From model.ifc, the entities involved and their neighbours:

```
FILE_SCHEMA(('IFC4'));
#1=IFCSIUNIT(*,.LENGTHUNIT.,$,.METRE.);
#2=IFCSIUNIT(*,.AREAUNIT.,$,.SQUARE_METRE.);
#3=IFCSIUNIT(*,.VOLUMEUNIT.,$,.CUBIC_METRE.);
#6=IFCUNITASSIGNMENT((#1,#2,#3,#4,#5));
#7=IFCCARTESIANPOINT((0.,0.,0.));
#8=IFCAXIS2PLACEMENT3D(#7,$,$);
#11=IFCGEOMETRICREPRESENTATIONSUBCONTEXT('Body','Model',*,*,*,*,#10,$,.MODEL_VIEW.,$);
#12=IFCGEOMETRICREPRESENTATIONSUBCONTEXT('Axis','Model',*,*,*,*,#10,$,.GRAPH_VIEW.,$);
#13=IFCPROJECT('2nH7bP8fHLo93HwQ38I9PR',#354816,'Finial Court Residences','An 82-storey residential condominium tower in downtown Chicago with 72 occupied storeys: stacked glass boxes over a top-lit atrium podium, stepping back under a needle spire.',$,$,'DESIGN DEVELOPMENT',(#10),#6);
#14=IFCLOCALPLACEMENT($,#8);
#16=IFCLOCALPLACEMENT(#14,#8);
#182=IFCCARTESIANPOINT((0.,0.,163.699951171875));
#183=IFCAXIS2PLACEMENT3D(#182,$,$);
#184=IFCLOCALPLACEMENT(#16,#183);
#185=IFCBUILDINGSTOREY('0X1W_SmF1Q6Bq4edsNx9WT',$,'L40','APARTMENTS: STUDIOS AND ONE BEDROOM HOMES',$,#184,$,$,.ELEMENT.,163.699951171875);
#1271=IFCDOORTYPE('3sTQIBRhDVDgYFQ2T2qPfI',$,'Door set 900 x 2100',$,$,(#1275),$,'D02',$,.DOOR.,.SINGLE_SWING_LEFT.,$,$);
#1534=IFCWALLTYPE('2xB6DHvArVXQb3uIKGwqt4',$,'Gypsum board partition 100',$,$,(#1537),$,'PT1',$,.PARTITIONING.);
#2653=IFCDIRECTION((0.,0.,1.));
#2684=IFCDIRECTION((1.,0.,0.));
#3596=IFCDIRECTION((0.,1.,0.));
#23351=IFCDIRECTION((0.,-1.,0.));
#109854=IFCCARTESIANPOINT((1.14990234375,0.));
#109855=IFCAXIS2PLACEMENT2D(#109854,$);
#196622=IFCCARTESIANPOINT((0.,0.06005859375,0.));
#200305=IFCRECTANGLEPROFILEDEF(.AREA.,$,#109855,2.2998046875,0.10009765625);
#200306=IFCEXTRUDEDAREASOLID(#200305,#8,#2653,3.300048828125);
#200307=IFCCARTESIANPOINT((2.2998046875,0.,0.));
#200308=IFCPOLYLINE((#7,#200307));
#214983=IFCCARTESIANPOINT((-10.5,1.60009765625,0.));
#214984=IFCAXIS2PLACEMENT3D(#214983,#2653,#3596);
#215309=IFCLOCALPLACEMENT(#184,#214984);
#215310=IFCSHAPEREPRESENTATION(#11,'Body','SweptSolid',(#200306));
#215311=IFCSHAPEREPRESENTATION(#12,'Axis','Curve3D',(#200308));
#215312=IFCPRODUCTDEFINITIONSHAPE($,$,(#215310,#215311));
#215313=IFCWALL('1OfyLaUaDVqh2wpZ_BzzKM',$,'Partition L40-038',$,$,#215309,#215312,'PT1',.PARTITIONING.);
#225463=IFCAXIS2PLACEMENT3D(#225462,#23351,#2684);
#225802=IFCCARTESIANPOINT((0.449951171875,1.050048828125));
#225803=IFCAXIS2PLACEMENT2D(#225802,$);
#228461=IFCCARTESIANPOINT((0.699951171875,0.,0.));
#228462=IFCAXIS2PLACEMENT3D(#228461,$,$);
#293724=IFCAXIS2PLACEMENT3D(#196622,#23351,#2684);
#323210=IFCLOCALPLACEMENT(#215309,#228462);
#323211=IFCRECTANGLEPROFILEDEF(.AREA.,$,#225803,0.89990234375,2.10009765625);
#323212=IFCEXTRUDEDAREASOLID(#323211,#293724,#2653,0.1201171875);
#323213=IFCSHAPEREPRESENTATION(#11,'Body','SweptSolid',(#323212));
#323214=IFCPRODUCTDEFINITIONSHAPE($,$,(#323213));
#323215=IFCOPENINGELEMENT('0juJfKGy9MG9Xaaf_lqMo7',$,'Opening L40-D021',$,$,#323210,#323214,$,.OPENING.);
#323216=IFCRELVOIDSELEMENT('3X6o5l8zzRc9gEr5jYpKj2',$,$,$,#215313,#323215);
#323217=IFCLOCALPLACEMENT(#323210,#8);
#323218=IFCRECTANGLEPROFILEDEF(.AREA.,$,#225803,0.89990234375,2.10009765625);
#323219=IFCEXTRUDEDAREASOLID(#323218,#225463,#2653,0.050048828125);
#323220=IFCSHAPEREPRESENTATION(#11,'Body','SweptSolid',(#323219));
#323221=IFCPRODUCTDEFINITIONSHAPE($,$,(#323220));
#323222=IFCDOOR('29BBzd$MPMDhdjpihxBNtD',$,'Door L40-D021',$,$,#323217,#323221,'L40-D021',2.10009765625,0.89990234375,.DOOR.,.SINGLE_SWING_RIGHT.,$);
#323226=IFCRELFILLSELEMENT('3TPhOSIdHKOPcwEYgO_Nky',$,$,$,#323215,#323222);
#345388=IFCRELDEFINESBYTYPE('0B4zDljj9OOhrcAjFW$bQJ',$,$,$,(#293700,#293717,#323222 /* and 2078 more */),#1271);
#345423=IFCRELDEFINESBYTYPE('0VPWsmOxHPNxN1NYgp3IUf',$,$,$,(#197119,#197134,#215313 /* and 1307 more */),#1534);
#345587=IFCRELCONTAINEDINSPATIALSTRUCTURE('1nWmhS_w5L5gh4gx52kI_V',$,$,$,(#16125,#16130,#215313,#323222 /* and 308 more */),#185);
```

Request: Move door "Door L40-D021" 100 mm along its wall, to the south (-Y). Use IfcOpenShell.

```python
import ifcopenshell
import ifcopenshell.api.geometry
import ifcopenshell.util.placement
import ifcopenshell.util.unit

model = ifcopenshell.open("model.ifc")
unit_scale = ifcopenshell.util.unit.calculate_unit_scale(model)

door = model.by_guid("29BBzd$MPMDhdjpihxBNtD")
opening = door.FillsVoids[0].RelatingOpeningElement
wall = opening.VoidsElements[0].RelatingBuildingElement

wall_matrix = ifcopenshell.util.placement.get_local_placement(wall.ObjectPlacement)
shift = wall_matrix[:3, 0] * -0.1 / unit_scale
before = ifcopenshell.util.placement.get_local_placement(door.ObjectPlacement)[:3, 3].copy()

# The door is placed relative to its opening, so it follows when the opening moves.
matrix = ifcopenshell.util.placement.get_local_placement(opening.ObjectPlacement)
matrix[:3, 3] += shift
ifcopenshell.api.geometry.edit_object_placement(
    model, product=opening, matrix=matrix, is_si=False, should_transform_children=True
)

after = ifcopenshell.util.placement.get_local_placement(door.ObjectPlacement)[:3, 3]
print("door moved by", (after - before).round(3) + 0.0)

model.write("model_v2.ifc")
```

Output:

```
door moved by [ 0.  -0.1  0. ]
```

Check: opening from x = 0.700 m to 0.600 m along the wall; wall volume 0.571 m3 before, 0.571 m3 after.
